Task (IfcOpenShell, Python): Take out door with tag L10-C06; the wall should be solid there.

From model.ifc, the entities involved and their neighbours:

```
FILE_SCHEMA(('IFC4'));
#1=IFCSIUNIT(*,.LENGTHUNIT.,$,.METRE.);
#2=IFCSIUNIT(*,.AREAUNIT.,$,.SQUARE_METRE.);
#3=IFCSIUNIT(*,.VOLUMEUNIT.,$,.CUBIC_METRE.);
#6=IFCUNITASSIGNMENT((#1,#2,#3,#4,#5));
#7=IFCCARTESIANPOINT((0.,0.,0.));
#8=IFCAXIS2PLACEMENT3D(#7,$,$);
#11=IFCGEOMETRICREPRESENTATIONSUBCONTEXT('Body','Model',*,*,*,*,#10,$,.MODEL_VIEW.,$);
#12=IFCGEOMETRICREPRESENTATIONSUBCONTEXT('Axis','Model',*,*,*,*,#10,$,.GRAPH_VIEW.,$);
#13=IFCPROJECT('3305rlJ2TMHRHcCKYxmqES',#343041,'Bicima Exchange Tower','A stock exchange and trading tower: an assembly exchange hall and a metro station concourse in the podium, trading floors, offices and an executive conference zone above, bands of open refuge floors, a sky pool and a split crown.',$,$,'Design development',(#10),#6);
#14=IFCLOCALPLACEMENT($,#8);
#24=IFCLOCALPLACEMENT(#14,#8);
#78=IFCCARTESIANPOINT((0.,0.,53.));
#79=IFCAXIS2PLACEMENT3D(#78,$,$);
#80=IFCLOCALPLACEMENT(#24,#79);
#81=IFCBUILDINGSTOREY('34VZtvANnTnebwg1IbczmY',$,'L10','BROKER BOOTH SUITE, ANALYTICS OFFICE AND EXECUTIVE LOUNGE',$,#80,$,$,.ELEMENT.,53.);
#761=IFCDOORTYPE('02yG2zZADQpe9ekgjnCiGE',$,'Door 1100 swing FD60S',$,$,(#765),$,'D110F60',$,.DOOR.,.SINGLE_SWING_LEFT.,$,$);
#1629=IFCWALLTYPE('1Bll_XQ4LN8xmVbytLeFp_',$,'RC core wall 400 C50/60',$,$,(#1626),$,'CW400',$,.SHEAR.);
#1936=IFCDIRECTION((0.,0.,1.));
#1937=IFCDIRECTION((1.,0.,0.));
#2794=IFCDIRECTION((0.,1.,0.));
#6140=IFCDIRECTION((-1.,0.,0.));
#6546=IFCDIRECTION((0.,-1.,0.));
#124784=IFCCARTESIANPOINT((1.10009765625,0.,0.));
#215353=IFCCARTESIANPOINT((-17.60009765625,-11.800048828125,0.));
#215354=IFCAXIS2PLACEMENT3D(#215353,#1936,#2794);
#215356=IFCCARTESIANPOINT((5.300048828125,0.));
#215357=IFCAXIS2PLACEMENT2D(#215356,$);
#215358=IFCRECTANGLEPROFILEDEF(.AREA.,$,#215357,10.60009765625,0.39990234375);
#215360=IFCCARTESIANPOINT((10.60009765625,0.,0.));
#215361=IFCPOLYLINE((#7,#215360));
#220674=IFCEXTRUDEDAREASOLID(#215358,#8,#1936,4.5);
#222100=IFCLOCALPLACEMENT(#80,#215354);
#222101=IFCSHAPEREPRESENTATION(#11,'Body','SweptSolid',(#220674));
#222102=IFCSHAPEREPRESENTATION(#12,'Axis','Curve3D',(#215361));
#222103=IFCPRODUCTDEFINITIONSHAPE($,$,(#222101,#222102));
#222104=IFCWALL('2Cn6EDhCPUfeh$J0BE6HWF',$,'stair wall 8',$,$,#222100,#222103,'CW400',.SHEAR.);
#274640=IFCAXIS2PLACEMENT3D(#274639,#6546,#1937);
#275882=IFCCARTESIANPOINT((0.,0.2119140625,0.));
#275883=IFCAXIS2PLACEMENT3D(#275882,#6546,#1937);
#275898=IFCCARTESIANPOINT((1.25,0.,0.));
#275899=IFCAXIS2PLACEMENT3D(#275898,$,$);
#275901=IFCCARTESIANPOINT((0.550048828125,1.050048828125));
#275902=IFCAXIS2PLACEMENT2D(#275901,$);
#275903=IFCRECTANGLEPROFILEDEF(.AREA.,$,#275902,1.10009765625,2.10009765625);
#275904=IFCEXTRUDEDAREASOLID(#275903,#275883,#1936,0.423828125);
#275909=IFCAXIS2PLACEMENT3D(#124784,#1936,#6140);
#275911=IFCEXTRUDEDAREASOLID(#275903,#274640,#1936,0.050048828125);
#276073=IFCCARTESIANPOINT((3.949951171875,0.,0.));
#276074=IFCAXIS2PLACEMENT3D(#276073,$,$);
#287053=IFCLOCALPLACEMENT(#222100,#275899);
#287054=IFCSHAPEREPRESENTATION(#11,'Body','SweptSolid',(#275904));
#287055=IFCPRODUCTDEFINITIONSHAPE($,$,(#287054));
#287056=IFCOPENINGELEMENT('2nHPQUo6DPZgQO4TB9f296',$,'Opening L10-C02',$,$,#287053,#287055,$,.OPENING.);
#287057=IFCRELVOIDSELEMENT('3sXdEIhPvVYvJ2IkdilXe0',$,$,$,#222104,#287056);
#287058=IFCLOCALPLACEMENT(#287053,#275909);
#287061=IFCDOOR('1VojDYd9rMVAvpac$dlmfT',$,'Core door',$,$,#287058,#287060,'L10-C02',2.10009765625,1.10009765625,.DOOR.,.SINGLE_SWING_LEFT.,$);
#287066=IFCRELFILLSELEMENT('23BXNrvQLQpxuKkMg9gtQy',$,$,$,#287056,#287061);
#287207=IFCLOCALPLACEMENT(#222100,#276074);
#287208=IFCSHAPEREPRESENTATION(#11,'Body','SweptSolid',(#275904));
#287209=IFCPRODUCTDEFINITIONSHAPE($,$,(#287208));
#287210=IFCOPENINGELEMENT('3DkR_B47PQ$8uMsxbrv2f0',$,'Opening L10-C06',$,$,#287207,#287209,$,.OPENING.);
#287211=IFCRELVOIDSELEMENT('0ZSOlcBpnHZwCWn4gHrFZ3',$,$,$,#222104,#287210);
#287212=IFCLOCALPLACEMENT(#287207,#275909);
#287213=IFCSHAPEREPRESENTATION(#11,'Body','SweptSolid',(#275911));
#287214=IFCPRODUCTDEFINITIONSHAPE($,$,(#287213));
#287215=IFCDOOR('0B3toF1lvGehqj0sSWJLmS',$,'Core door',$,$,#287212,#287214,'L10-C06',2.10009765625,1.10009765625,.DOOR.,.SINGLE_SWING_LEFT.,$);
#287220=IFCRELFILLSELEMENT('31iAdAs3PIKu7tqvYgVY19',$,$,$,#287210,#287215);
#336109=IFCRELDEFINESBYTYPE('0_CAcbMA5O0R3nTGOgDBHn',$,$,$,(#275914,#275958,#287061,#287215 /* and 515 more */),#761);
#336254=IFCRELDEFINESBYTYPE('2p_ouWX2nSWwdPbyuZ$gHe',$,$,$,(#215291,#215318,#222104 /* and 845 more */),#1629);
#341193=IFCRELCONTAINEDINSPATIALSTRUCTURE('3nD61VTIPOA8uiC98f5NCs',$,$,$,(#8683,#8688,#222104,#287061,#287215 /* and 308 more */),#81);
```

```python
import ifcopenshell
import ifcopenshell.api.feature
import ifcopenshell.api.root
import ifcopenshell.geom
import ifcopenshell.util.shape

model = ifcopenshell.open("model.ifc")
settings = ifcopenshell.geom.settings()


def volume(element):
    """Net volume in cubic metres, openings subtracted."""
    shape = ifcopenshell.geom.create_shape(settings, element)
    return ifcopenshell.util.shape.get_volume(shape.geometry)


door = model.by_guid("0B3toF1lvGehqj0sSWJLmS")
opening = door.FillsVoids[0].RelatingOpeningElement
wall = opening.VoidsElements[0].RelatingBuildingElement
before = volume(wall)

ifcopenshell.api.root.remove_product(model, product=door)
ifcopenshell.api.feature.remove_feature(model, feature=opening)

after = volume(wall)

print(f"wall volume {before:.3f} -> {after:.3f} m3")

model.write("model_v2.ifc")
```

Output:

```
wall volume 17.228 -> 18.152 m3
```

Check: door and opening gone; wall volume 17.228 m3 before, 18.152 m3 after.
